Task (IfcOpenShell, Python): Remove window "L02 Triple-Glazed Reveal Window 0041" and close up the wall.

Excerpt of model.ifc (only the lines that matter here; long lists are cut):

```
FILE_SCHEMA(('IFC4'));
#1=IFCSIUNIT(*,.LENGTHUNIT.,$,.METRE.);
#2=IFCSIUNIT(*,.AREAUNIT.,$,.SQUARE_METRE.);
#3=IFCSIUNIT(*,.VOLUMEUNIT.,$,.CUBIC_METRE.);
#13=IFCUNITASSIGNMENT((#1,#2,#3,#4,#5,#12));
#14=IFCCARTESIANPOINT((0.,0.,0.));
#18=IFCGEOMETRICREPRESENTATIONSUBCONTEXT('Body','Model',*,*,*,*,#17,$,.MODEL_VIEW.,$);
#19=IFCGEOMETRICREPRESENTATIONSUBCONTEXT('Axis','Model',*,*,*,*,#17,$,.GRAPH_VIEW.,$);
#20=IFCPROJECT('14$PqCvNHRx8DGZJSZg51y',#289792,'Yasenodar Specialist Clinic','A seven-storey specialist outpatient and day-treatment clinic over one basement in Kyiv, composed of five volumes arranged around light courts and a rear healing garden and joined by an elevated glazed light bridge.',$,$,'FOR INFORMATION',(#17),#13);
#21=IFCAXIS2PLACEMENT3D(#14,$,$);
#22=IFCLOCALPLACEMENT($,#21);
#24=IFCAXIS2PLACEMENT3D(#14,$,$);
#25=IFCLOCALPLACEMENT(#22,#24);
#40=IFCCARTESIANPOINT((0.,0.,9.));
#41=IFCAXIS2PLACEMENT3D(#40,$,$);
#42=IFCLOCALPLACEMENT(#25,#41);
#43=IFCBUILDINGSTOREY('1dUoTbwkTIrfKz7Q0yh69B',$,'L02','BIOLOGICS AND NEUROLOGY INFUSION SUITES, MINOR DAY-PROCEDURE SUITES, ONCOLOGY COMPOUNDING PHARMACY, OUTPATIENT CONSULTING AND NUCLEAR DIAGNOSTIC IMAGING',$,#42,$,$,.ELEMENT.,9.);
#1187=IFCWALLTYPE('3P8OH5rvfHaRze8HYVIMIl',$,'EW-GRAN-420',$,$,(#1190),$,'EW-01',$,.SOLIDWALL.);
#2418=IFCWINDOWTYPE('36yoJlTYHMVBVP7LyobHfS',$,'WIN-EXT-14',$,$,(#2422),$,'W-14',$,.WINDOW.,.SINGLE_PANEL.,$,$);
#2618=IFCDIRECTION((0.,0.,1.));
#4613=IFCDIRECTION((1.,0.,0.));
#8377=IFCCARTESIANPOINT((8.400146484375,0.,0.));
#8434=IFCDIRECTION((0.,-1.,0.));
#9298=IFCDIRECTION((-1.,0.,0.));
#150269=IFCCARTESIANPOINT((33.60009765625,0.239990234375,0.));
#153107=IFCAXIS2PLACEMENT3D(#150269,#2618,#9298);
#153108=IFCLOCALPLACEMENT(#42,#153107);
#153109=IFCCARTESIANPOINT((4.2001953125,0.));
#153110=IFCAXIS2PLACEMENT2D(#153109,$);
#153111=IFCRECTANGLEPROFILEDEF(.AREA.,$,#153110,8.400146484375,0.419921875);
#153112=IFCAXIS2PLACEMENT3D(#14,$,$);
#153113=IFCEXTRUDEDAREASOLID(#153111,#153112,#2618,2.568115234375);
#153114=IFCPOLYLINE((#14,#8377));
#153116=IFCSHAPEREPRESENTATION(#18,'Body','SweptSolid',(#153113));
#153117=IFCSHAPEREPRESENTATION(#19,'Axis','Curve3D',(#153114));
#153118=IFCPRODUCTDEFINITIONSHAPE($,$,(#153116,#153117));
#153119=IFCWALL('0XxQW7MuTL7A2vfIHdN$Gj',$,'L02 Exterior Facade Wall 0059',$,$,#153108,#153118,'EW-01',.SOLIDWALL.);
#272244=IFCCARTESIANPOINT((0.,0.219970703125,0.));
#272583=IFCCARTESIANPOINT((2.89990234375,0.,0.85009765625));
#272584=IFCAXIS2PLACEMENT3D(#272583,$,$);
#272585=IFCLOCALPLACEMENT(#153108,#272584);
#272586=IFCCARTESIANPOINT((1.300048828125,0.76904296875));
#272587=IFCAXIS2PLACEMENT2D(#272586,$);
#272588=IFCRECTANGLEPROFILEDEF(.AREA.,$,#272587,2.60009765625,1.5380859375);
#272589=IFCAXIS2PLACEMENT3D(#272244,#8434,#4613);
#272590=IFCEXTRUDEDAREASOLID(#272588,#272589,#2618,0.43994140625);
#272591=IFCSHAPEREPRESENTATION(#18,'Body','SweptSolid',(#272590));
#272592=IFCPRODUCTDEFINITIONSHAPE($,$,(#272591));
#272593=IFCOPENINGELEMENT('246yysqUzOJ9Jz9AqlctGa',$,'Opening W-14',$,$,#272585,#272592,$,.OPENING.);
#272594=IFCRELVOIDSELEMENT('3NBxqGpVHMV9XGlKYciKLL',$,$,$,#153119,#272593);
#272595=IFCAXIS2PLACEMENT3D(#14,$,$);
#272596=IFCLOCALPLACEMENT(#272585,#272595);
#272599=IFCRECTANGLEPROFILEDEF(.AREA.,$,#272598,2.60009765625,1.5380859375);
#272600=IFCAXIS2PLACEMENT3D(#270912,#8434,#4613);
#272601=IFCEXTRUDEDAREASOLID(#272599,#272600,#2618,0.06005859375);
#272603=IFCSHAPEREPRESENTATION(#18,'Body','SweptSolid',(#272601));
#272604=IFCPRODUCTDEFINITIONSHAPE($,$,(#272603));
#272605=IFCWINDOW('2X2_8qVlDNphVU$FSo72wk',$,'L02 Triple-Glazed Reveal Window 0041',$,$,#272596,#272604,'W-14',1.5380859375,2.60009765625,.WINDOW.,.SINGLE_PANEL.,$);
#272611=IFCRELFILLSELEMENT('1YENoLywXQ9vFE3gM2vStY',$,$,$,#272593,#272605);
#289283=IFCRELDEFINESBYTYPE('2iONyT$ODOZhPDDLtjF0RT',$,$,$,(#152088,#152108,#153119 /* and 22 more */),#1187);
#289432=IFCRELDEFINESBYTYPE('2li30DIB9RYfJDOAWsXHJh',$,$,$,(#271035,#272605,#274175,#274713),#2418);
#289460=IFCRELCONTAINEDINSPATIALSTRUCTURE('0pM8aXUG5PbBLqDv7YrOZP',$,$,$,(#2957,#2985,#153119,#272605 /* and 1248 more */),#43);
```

```python
import ifcopenshell
import ifcopenshell.api.feature
import ifcopenshell.api.root
import ifcopenshell.geom
import ifcopenshell.util.shape

model = ifcopenshell.open("model.ifc")
settings = ifcopenshell.geom.settings()


def volume(element):
    """Net volume in cubic metres, openings subtracted."""
    shape = ifcopenshell.geom.create_shape(settings, element)
    return ifcopenshell.util.shape.get_volume(shape.geometry)


window = model.by_guid("2X2_8qVlDNphVU$FSo72wk")
opening = window.FillsVoids[0].RelatingOpeningElement
wall = opening.VoidsElements[0].RelatingBuildingElement
before = volume(wall)

ifcopenshell.api.root.remove_product(model, product=window)
ifcopenshell.api.feature.remove_feature(model, feature=opening)

after = volume(wall)

print(f"wall volume {before:.3f} -> {after:.3f} m3")

model.write("model_rev.ifc")
```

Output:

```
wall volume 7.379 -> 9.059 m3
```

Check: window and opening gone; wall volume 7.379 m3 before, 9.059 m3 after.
